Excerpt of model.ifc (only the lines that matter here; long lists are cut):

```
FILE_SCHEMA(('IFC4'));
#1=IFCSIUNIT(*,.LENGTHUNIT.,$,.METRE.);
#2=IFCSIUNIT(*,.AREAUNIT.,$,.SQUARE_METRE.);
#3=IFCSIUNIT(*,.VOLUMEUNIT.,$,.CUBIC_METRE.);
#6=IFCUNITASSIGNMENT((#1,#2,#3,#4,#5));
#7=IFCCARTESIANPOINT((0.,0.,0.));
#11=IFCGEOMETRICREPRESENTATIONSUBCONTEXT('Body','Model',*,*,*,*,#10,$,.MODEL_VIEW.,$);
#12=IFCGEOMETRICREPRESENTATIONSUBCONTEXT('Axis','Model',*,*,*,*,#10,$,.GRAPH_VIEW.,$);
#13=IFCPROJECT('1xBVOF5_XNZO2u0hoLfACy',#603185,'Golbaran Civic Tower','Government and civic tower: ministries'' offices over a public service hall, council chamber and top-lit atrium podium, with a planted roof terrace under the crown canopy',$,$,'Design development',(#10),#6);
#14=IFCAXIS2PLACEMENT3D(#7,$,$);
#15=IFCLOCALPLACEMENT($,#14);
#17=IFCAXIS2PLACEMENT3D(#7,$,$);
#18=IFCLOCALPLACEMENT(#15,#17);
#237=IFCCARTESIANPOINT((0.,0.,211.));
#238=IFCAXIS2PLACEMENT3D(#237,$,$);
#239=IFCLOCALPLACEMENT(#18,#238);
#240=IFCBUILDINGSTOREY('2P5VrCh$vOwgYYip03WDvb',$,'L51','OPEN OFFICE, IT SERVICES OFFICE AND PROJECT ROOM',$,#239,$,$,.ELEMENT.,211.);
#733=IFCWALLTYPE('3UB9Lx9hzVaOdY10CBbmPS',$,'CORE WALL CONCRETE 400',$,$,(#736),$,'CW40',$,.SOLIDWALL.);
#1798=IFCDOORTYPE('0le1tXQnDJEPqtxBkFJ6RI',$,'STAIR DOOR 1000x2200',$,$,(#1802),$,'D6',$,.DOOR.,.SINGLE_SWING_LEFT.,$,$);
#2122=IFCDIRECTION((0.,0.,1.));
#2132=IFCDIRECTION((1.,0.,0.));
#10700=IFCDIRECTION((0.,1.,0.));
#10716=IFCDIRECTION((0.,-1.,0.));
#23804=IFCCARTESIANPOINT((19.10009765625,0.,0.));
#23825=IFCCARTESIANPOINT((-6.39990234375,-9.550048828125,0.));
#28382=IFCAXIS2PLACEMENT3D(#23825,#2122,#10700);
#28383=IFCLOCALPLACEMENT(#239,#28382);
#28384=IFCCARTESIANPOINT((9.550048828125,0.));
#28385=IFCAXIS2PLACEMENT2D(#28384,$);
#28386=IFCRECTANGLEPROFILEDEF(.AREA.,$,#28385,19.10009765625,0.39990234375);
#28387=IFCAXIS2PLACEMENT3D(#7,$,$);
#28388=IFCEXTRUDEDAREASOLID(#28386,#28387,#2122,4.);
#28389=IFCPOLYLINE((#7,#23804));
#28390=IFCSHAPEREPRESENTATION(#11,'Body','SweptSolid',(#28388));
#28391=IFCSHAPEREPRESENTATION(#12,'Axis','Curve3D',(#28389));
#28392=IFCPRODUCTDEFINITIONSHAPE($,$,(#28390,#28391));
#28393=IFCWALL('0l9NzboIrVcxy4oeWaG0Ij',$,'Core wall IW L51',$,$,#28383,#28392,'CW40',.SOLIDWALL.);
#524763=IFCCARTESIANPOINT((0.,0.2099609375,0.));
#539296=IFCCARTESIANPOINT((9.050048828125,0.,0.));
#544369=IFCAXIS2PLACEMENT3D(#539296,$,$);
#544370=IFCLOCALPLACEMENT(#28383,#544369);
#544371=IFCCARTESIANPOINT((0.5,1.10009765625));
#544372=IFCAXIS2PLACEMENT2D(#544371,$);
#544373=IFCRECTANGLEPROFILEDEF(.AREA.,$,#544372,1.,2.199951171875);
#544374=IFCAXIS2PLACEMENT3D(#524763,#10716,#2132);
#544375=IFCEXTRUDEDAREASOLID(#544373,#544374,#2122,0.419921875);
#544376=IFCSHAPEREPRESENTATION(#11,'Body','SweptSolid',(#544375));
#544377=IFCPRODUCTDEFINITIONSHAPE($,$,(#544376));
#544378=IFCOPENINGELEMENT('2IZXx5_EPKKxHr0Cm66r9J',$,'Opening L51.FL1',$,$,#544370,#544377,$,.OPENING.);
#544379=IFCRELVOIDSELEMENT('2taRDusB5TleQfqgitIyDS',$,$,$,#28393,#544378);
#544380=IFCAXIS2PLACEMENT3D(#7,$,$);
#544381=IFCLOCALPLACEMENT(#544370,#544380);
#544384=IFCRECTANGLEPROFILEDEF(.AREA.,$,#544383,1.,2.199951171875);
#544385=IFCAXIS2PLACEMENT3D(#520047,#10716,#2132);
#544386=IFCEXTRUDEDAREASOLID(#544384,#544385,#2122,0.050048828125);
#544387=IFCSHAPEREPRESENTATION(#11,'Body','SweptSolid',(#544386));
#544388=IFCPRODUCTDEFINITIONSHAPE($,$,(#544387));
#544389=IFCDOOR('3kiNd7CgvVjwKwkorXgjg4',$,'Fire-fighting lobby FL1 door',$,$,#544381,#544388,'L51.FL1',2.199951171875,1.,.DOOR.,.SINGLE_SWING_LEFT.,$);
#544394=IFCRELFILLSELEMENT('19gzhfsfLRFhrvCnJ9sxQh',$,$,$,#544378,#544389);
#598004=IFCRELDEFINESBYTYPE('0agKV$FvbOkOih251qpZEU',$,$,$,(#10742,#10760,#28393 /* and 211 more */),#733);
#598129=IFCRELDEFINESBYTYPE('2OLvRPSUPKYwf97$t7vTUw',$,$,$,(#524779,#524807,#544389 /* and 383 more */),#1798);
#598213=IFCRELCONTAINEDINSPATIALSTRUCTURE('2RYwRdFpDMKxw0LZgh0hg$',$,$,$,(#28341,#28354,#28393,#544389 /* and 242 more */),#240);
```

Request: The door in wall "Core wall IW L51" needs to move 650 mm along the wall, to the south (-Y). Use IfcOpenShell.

```python
import ifcopenshell
import ifcopenshell.api.geometry
import ifcopenshell.util.placement
import ifcopenshell.util.unit

model = ifcopenshell.open("model.ifc")
unit_scale = ifcopenshell.util.unit.calculate_unit_scale(model)

door = model.by_guid("3kiNd7CgvVjwKwkorXgjg4")
opening = door.FillsVoids[0].RelatingOpeningElement
wall = opening.VoidsElements[0].RelatingBuildingElement

wall_matrix = ifcopenshell.util.placement.get_local_placement(wall.ObjectPlacement)
shift = wall_matrix[:3, 0] * -0.65 / unit_scale
before = ifcopenshell.util.placement.get_local_placement(door.ObjectPlacement)[:3, 3].copy()

# The door is placed relative to its opening, so it follows when the opening moves.
matrix = ifcopenshell.util.placement.get_local_placement(opening.ObjectPlacement)
matrix[:3, 3] += shift
ifcopenshell.api.geometry.edit_object_placement(
    model, product=opening, matrix=matrix, is_si=False, should_transform_children=True
)

after = ifcopenshell.util.placement.get_local_placement(door.ObjectPlacement)[:3, 3]
print("door moved by", (after - before).round(3) + 0.0)

model.write("model_edited.ifc")
```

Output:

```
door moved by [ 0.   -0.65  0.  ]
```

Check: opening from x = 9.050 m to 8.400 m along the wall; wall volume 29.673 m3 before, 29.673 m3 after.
